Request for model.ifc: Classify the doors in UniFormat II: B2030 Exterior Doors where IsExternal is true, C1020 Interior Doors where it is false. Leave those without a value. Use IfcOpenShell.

First a look at what the model holds.

```python
import ifcopenshell
import ifcopenshell.util.element

model = ifcopenshell.open("model.ifc")
print(model.schema)
print("classifications:", [c.Name for c in model.by_type("IfcClassification")])
values = [ifcopenshell.util.element.get_pset(e, "Pset_DoorCommon", "IsExternal") for e in model.by_type("IfcDoor")]
for value in (True, False, None):
    print("IsExternal", value, values.count(value))
```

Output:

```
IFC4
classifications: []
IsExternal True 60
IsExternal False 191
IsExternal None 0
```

```python
import ifcopenshell
import ifcopenshell.api.classification
import ifcopenshell.util.element

model = ifcopenshell.open("model.ifc")

system = ifcopenshell.api.classification.add_classification(model, classification="UniFormat II")

doors = model.by_type("IfcDoor")
external = {e: ifcopenshell.util.element.get_pset(e, "Pset_DoorCommon", "IsExternal") for e in doors}
for flag, code, name in ((True, "B2030", "Exterior Doors"), (False, "C1020", "Interior Doors")):
    products = [e for e in doors if external[e] is flag]
    ifcopenshell.api.classification.add_reference(
        model, products=products, classification=system, identification=code, name=name
    )
    print(code, len(products))

model.write("model_v2.ifc")
```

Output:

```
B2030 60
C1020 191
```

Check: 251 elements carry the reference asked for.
